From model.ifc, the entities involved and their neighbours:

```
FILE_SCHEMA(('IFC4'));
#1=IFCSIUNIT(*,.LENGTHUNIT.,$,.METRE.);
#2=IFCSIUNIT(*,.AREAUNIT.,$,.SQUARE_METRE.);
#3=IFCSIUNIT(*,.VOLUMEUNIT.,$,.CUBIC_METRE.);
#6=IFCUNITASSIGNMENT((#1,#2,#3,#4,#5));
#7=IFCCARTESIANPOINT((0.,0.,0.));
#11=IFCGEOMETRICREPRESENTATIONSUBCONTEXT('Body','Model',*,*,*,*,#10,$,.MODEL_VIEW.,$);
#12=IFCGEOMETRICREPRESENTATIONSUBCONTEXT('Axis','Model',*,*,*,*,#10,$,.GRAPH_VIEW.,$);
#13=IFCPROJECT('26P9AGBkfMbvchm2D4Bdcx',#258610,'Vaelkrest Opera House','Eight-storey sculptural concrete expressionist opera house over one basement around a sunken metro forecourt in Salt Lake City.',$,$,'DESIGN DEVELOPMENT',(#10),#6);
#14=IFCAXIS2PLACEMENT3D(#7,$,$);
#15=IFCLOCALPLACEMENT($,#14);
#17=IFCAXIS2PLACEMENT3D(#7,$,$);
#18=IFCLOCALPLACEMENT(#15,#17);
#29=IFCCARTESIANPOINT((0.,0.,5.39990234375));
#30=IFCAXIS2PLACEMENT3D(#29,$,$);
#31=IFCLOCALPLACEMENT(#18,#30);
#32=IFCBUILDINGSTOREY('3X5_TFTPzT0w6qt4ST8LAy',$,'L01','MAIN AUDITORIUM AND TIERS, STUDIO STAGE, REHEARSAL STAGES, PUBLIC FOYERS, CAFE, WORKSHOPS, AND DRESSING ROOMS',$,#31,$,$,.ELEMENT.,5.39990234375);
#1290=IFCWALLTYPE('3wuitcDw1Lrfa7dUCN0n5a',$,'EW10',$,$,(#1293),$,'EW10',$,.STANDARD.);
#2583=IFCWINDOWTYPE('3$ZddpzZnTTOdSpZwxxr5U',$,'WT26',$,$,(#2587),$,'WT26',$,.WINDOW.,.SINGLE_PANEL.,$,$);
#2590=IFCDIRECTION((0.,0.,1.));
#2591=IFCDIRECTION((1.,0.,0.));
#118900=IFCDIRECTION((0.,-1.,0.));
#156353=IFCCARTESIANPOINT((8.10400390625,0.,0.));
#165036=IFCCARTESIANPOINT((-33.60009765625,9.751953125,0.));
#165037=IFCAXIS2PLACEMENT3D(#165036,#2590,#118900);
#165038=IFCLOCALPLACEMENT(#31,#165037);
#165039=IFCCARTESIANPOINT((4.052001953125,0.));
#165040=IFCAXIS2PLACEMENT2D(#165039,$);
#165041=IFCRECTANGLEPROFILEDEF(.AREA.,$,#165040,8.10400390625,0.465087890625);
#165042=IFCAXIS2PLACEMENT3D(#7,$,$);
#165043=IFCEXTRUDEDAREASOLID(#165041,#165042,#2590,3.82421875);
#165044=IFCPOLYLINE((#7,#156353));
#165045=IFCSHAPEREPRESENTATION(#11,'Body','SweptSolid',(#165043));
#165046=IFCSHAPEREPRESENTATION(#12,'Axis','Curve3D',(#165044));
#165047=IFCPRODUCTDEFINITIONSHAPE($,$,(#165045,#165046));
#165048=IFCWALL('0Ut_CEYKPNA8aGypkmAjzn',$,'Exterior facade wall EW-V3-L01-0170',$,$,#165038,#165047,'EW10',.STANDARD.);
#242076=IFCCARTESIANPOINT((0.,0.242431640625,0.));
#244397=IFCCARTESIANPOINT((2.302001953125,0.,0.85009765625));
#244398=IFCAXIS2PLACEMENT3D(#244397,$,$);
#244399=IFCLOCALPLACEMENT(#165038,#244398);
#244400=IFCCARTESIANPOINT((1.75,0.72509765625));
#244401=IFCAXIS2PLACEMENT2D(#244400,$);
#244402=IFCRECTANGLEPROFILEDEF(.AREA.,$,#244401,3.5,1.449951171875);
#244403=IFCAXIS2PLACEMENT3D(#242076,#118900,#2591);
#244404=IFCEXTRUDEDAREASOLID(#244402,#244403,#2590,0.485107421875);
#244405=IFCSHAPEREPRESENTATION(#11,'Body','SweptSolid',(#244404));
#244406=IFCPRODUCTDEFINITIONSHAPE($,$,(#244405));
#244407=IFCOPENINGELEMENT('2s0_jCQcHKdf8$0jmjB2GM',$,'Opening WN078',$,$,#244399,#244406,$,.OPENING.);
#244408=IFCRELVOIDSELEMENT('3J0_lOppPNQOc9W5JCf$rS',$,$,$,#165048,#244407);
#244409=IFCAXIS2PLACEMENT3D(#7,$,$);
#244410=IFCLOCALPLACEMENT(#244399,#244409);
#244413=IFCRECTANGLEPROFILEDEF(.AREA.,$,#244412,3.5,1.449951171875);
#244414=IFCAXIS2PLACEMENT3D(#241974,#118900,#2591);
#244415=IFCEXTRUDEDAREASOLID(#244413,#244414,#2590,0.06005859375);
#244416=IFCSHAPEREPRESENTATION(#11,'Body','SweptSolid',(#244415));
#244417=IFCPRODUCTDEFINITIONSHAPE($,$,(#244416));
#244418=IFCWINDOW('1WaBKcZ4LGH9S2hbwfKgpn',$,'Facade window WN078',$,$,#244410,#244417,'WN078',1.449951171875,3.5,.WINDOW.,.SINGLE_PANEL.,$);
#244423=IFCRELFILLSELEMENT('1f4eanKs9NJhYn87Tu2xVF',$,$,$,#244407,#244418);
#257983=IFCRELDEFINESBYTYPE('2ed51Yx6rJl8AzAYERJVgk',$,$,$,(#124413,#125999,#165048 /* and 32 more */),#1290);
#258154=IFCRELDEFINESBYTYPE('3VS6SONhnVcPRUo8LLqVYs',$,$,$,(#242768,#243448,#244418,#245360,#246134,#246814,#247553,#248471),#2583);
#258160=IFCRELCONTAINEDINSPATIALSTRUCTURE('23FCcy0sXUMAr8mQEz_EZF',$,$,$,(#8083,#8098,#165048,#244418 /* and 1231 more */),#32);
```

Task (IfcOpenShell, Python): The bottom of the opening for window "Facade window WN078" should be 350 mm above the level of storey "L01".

```python
import numpy as np
import ifcopenshell
import ifcopenshell.api.geometry
import ifcopenshell.geom
import ifcopenshell.util.element
import ifcopenshell.util.placement
import ifcopenshell.util.shape
import ifcopenshell.util.unit

model = ifcopenshell.open("model.ifc")
unit_scale = ifcopenshell.util.unit.calculate_unit_scale(model)

window = model.by_id(244418)
opening = window.FillsVoids[0].RelatingOpeningElement
storey = ifcopenshell.util.element.get_container(window, ifc_class="IfcBuildingStorey")
level = ifcopenshell.util.placement.get_local_placement(storey.ObjectPlacement)[2, 3]

# The opening's origin need not be at the sill, so measure its lowest point.
shape = ifcopenshell.geom.create_shape(ifcopenshell.geom.settings(), opening)
bottom = ifcopenshell.util.shape.get_shape_bottom_elevation(shape, shape.geometry) / unit_scale
dz = level + 0.35 / unit_scale - bottom

shift = np.array([0.0, 0.0, dz])
# The window is placed relative to its opening, so it follows when the opening moves.
matrix = ifcopenshell.util.placement.get_local_placement(opening.ObjectPlacement)
matrix[:3, 3] += shift
ifcopenshell.api.geometry.edit_object_placement(
    model, product=opening, matrix=matrix, is_si=False, should_transform_children=True
)

print(f"moved by {dz * unit_scale:+.3f} m")

model.write("model-out.ifc")
```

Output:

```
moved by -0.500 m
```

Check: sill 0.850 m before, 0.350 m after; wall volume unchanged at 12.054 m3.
